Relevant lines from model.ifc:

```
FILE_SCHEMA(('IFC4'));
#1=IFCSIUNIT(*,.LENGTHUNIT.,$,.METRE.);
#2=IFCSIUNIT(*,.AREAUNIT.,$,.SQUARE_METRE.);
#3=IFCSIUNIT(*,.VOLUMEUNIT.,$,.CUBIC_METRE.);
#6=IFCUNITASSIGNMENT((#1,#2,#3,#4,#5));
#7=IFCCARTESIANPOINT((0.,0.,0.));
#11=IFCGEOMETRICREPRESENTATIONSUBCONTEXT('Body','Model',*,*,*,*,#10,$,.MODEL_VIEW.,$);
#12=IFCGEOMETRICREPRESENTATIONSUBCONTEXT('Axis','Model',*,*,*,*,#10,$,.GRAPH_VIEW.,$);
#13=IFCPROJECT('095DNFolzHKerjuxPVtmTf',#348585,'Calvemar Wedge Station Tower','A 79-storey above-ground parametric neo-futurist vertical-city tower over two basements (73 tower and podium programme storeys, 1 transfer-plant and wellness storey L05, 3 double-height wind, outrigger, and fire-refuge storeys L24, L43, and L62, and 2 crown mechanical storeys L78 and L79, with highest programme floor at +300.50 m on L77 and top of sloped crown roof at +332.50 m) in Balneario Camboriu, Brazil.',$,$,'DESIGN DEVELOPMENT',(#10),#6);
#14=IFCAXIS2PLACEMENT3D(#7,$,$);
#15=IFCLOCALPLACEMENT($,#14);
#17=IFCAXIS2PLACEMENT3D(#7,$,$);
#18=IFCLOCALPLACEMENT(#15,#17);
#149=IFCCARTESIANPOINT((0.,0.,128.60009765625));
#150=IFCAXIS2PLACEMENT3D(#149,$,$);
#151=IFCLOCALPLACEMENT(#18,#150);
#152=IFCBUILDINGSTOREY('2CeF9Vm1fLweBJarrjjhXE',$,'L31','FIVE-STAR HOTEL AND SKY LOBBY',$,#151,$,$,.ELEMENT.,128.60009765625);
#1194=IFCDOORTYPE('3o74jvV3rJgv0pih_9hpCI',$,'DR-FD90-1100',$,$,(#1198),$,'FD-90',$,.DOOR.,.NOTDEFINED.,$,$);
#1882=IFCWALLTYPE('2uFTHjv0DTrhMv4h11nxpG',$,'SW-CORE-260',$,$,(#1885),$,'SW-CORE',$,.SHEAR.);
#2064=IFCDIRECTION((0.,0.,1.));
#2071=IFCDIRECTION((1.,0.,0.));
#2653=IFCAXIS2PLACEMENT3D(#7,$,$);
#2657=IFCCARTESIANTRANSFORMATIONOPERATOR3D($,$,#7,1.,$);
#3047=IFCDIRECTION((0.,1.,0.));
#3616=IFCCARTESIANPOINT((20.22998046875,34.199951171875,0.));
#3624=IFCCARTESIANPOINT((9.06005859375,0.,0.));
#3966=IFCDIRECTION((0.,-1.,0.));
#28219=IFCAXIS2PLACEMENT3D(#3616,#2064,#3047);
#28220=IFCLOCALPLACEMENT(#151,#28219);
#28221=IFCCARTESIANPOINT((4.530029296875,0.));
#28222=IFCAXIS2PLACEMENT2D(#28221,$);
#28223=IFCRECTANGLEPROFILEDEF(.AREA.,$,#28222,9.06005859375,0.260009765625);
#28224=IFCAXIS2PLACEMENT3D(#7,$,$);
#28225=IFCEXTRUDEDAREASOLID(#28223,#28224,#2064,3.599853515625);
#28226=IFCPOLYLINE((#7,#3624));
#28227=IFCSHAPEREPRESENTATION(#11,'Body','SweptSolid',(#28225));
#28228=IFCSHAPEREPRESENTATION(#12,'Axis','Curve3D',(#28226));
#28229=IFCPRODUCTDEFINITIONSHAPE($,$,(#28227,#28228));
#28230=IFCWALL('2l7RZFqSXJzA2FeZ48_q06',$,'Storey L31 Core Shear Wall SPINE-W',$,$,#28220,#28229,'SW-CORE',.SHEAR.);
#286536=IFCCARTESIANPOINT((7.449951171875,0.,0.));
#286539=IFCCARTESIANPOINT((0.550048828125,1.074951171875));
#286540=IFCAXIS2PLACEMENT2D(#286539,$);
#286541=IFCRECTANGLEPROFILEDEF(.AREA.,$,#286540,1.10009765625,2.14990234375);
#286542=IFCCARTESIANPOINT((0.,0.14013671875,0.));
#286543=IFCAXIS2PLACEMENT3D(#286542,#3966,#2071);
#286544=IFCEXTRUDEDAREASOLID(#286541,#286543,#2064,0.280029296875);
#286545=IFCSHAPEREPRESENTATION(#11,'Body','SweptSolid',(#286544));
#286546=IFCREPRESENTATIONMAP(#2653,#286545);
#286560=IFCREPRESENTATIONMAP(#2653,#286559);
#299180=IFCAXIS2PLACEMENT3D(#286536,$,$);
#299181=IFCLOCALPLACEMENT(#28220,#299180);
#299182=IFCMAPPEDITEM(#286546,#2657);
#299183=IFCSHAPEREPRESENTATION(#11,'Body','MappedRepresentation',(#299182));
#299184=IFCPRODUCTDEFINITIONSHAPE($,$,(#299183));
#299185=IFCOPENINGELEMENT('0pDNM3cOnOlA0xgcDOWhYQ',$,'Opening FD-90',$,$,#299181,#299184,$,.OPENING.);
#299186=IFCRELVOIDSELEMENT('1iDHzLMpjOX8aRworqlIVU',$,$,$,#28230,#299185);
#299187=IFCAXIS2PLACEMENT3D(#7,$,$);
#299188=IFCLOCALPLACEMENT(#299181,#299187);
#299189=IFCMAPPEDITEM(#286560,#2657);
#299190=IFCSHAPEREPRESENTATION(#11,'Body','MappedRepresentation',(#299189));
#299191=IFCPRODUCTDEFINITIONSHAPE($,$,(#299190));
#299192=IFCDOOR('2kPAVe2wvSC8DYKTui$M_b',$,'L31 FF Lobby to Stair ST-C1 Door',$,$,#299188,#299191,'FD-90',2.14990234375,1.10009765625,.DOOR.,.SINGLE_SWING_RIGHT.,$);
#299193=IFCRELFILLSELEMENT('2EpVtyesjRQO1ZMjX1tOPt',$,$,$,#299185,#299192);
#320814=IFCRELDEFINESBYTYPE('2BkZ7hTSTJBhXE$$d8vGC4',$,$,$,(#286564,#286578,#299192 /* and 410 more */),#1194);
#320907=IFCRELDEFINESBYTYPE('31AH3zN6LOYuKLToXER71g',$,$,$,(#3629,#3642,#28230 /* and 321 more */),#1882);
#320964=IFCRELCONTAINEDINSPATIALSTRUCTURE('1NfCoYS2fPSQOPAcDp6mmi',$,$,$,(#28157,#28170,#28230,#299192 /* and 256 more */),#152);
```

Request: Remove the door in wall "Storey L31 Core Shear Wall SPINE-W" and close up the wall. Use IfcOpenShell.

```python
import ifcopenshell
import ifcopenshell.api.feature
import ifcopenshell.api.root
import ifcopenshell.geom
import ifcopenshell.util.shape

model = ifcopenshell.open("model.ifc")
settings = ifcopenshell.geom.settings()


def volume(element):
    """Net volume in cubic metres, openings subtracted."""
    shape = ifcopenshell.geom.create_shape(settings, element)
    return ifcopenshell.util.shape.get_volume(shape.geometry)


door = model.by_id(299192)
opening = door.FillsVoids[0].RelatingOpeningElement
wall = opening.VoidsElements[0].RelatingBuildingElement
before = volume(wall)

ifcopenshell.api.root.remove_product(model, product=door)
ifcopenshell.api.feature.remove_feature(model, feature=opening)

after = volume(wall)

print(f"wall volume {before:.3f} -> {after:.3f} m3")

model.write("model-out.ifc")
```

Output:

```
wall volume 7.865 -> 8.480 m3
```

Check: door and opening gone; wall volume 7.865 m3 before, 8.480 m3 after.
